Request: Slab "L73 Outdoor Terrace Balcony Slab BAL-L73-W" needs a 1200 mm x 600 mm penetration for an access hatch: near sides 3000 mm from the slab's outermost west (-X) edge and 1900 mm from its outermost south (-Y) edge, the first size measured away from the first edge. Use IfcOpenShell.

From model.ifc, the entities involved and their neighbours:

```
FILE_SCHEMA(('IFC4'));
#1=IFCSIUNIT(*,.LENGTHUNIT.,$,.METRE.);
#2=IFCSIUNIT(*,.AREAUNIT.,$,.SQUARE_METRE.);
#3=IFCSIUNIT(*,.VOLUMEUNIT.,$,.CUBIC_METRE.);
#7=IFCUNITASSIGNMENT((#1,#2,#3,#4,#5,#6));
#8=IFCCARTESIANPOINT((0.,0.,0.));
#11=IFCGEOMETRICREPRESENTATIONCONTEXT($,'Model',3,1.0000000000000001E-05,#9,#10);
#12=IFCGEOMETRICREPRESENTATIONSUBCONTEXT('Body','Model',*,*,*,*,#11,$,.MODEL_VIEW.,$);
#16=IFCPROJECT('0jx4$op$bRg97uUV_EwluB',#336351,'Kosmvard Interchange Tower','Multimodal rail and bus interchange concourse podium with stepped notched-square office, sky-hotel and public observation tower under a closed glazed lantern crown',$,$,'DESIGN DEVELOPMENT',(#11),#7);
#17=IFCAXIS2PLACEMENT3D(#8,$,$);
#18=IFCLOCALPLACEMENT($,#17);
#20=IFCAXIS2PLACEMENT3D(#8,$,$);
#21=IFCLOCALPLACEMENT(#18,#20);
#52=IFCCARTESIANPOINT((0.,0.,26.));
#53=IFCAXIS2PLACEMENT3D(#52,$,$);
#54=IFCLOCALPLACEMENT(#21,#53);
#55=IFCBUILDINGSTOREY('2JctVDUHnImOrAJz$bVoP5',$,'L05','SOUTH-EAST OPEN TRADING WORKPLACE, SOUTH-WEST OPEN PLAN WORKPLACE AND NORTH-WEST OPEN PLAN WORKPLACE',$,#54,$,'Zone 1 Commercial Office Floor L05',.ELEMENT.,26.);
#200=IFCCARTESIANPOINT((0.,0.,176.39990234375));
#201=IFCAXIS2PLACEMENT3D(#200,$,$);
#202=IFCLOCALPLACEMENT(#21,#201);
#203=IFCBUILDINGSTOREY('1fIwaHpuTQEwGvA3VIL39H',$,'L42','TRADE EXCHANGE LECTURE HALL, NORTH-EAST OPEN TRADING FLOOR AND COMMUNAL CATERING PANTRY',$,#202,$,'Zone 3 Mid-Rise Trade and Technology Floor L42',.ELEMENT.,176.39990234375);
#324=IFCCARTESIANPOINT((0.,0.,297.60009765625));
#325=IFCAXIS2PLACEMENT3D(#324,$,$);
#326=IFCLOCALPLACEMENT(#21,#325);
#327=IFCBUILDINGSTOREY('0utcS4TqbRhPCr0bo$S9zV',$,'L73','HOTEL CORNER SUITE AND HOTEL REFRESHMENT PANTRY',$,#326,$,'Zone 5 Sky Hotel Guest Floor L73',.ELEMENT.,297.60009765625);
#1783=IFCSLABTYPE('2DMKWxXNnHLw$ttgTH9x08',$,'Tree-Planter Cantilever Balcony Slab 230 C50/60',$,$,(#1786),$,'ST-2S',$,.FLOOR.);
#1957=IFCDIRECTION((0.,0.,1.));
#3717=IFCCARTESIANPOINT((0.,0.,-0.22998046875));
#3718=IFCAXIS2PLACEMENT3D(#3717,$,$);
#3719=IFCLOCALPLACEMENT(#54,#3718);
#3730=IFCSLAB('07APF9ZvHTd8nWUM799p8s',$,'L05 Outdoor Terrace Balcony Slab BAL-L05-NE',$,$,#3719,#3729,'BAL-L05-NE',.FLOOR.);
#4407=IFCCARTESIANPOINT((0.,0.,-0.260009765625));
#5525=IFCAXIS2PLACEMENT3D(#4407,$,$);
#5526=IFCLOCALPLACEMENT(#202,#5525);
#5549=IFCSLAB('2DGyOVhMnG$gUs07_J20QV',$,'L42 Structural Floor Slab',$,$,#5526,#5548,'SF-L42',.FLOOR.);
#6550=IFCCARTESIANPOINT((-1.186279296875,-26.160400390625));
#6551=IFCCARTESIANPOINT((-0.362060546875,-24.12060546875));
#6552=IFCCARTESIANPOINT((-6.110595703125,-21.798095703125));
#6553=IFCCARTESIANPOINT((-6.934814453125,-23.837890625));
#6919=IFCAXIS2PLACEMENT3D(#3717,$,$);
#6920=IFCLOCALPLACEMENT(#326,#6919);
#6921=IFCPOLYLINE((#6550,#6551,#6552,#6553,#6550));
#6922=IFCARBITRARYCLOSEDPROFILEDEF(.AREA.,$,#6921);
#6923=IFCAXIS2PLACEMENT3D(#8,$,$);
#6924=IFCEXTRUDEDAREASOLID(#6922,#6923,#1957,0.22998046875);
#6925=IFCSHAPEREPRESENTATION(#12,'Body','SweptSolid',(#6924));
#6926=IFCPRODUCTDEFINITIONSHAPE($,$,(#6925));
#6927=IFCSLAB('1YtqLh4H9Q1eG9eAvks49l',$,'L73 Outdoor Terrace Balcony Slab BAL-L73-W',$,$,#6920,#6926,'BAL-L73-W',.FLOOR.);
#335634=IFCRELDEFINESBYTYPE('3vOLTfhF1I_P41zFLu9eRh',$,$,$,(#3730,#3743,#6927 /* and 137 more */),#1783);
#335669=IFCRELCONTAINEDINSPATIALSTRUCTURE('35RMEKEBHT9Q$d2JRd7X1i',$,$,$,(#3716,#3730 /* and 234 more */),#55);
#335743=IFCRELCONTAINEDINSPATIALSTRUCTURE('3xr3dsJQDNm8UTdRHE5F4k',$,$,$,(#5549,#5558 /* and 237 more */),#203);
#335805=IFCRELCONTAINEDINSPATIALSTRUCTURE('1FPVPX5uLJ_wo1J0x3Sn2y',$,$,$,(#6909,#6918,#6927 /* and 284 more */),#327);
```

```python
import numpy as np
import ifcopenshell
import ifcopenshell.api.feature
import ifcopenshell.api.geometry
import ifcopenshell.api.root
import ifcopenshell.geom
import ifcopenshell.util.placement
import ifcopenshell.util.representation
import ifcopenshell.util.shape
import ifcopenshell.util.unit

model = ifcopenshell.open("model.ifc")
unit_scale = ifcopenshell.util.unit.calculate_unit_scale(model)
settings = ifcopenshell.geom.settings()


def volume(element):
    """Net volume in cubic metres, openings subtracted."""
    shape = ifcopenshell.geom.create_shape(settings, element)
    return ifcopenshell.util.shape.get_volume(shape.geometry)


slab = model.by_guid("1YtqLh4H9Q1eG9eAvks49l")
before = volume(slab)

# Extent in the slab's own axes, in metres. The edges named are its -X and -Y sides.
slab_shape = ifcopenshell.geom.create_shape(settings, slab)
vertices = ifcopenshell.util.shape.get_vertices(slab_shape.geometry)
x_min, y_min, bottom = vertices.min(axis=0)
top = vertices[:, 2].max()

opening = ifcopenshell.api.root.create_entity(model, ifc_class="IfcOpeningElement", name="Access hatch opening", predefined_type="OPENING")
context = ifcopenshell.util.representation.get_context(model, "Model", "Body", "MODEL_VIEW")
width, depth = 1.2, 0.6
outline = [(0.0, 0.0), (width, 0.0), (width, depth), (0.0, depth), (0.0, 0.0)]
# Overshoot both faces by 50 mm so the cut is clean.
shape = ifcopenshell.api.geometry.add_slab_representation(
    model, context=context, depth=top - bottom + 0.1, polyline=outline
)
ifcopenshell.api.geometry.assign_representation(model, product=opening, representation=shape)

matrix = ifcopenshell.util.placement.get_local_placement(slab.ObjectPlacement)
matrix[:, 3] = matrix @ np.append(np.array([x_min + 3, y_min + 1.9, bottom - 0.05]) / unit_scale, 1.0)
ifcopenshell.api.geometry.edit_object_placement(model, product=opening, matrix=matrix, is_si=False)
ifcopenshell.api.feature.add_feature(model, feature=opening, element=slab)

after = volume(slab)

print(f"slab volume {before:.3f} -> {after:.3f} m3")

model.write("model_updated.ifc")
```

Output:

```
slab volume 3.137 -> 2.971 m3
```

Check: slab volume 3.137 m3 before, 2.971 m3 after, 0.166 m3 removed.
